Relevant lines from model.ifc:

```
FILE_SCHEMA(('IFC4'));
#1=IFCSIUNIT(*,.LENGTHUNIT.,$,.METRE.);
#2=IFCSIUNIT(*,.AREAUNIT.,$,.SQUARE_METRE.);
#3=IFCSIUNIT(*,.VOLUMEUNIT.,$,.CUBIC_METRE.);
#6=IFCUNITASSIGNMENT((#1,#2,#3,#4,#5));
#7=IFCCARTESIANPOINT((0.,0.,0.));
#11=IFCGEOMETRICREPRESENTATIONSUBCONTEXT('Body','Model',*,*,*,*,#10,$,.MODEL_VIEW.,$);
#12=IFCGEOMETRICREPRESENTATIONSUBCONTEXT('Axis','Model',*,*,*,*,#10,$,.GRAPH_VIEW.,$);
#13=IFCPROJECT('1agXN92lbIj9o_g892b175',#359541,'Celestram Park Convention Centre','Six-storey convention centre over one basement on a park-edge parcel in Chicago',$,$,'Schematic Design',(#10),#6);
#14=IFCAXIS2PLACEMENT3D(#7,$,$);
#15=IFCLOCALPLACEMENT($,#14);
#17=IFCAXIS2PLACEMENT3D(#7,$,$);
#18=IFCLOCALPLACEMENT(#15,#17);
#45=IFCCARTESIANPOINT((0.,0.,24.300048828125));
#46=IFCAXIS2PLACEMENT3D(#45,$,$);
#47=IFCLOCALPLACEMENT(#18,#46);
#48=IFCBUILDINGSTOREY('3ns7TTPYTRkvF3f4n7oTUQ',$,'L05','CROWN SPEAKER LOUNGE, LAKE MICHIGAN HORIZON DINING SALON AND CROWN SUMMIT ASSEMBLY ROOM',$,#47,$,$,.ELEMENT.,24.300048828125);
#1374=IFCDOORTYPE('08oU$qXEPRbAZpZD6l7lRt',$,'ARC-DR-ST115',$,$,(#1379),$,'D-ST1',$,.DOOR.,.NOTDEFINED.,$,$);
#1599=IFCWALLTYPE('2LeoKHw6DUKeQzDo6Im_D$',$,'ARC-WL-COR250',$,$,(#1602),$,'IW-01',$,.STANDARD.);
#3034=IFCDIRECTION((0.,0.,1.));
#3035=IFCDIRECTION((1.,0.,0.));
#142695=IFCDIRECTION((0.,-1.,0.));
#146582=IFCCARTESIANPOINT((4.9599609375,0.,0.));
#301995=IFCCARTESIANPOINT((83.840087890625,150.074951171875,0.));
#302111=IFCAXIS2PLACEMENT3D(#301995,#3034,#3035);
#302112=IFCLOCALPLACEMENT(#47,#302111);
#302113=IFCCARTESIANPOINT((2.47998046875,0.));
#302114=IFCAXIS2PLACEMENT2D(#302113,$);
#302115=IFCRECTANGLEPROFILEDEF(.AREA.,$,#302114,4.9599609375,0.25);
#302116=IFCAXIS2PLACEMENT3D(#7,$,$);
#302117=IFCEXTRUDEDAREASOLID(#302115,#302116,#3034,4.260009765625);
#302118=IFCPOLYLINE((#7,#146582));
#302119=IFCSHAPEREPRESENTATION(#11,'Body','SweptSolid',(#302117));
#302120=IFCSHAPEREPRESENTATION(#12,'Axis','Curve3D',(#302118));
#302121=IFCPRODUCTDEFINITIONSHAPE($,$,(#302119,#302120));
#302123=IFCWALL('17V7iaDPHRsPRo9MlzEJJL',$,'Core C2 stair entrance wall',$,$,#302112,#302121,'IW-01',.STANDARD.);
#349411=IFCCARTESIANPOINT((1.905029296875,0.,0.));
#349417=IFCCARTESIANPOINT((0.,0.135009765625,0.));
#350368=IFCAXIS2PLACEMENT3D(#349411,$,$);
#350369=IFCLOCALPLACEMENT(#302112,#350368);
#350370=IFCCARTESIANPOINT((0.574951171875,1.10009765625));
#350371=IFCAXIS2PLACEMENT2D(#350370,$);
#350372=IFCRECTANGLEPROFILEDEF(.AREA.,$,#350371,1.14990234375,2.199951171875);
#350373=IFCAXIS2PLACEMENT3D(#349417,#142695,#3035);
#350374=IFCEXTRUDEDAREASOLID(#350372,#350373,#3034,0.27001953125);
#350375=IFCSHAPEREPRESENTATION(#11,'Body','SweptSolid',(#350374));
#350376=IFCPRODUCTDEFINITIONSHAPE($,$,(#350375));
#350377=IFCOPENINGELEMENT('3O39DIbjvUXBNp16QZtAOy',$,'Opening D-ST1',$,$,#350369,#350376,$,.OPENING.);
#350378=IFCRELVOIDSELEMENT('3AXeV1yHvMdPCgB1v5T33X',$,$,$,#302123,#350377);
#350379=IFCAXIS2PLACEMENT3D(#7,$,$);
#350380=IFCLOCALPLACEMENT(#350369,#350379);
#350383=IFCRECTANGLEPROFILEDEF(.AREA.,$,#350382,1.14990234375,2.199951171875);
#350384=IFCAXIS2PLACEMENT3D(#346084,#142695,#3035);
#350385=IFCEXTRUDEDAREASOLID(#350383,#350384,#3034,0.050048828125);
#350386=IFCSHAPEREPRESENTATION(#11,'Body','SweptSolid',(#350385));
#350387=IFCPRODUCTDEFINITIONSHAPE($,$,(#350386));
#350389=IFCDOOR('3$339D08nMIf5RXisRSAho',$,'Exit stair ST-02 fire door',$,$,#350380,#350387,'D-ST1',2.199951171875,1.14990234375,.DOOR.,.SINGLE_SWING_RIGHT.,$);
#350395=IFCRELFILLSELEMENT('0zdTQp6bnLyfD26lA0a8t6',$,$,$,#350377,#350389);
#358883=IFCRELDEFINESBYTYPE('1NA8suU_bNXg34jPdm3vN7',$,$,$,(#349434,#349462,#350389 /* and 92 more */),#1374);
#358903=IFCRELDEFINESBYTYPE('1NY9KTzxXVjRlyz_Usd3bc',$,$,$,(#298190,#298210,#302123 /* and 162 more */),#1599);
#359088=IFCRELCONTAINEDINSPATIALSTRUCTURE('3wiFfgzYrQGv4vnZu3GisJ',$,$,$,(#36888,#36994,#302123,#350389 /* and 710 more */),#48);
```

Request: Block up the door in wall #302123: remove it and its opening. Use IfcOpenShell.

```python
import ifcopenshell
import ifcopenshell.api.feature
import ifcopenshell.api.root
import ifcopenshell.geom
import ifcopenshell.util.shape

model = ifcopenshell.open("model.ifc")
settings = ifcopenshell.geom.settings()


def volume(element):
    """Net volume in cubic metres, openings subtracted."""
    shape = ifcopenshell.geom.create_shape(settings, element)
    return ifcopenshell.util.shape.get_volume(shape.geometry)


door = model.by_id(350389)
opening = door.FillsVoids[0].RelatingOpeningElement
wall = opening.VoidsElements[0].RelatingBuildingElement
before = volume(wall)

ifcopenshell.api.root.remove_product(model, product=door)
ifcopenshell.api.feature.remove_feature(model, feature=opening)

after = volume(wall)

print(f"wall volume {before:.3f} -> {after:.3f} m3")

model.write("model_v2.ifc")
```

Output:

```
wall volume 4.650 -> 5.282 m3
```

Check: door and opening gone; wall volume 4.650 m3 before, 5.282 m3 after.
